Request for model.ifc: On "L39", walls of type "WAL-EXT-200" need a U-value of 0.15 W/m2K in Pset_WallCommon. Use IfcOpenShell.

First a look at what the model holds.

```python
import ifcopenshell
import ifcopenshell.util.element

model = ifcopenshell.open("model.ifc")
print(model.schema)
storey = next(s for s in model.by_type("IfcBuildingStorey") if s.Name == "L39")
walls = [e for e in ifcopenshell.util.element.get_decomposition(storey) if e.is_a("IfcWall")]
seen = {}
for e in walls:
    element_type = ifcopenshell.util.element.get_type(e)
    key = (element_type.Name if element_type != e and element_type else None, ifcopenshell.util.element.get_pset(e, "Pset_WallCommon", "ThermalTransmittance"))
    seen[key] = seen.get(key, 0) + 1
for (name, value), count in sorted(seen.items(), key=str):
    print(count, "x", name, "|", value)
```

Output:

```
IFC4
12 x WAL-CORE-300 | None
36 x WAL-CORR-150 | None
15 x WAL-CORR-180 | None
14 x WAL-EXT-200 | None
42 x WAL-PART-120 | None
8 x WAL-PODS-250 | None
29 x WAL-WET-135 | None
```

```python
import ifcopenshell
import ifcopenshell.api.pset
import ifcopenshell.util.element

model = ifcopenshell.open("model.ifc")

storey = next(s for s in model.by_type("IfcBuildingStorey") if s.Name == "L39")
walls = [e for e in ifcopenshell.util.element.get_decomposition(storey) if e.is_a("IfcWall")]

count = 0
for e in walls:
    element_type = ifcopenshell.util.element.get_type(e)
    if element_type in (None, e) or element_type.Name != "WAL-EXT-200":
        continue
    # add_pset returns the element's existing set when there is one.
    pset = ifcopenshell.api.pset.add_pset(model, product=e, name="Pset_WallCommon")
    ifcopenshell.api.pset.edit_pset(model, pset=pset, properties={"ThermalTransmittance": 0.15})
    count += 1

print(count, "walls updated")

model.write("model_rev.ifc")
```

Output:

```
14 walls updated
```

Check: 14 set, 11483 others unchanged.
